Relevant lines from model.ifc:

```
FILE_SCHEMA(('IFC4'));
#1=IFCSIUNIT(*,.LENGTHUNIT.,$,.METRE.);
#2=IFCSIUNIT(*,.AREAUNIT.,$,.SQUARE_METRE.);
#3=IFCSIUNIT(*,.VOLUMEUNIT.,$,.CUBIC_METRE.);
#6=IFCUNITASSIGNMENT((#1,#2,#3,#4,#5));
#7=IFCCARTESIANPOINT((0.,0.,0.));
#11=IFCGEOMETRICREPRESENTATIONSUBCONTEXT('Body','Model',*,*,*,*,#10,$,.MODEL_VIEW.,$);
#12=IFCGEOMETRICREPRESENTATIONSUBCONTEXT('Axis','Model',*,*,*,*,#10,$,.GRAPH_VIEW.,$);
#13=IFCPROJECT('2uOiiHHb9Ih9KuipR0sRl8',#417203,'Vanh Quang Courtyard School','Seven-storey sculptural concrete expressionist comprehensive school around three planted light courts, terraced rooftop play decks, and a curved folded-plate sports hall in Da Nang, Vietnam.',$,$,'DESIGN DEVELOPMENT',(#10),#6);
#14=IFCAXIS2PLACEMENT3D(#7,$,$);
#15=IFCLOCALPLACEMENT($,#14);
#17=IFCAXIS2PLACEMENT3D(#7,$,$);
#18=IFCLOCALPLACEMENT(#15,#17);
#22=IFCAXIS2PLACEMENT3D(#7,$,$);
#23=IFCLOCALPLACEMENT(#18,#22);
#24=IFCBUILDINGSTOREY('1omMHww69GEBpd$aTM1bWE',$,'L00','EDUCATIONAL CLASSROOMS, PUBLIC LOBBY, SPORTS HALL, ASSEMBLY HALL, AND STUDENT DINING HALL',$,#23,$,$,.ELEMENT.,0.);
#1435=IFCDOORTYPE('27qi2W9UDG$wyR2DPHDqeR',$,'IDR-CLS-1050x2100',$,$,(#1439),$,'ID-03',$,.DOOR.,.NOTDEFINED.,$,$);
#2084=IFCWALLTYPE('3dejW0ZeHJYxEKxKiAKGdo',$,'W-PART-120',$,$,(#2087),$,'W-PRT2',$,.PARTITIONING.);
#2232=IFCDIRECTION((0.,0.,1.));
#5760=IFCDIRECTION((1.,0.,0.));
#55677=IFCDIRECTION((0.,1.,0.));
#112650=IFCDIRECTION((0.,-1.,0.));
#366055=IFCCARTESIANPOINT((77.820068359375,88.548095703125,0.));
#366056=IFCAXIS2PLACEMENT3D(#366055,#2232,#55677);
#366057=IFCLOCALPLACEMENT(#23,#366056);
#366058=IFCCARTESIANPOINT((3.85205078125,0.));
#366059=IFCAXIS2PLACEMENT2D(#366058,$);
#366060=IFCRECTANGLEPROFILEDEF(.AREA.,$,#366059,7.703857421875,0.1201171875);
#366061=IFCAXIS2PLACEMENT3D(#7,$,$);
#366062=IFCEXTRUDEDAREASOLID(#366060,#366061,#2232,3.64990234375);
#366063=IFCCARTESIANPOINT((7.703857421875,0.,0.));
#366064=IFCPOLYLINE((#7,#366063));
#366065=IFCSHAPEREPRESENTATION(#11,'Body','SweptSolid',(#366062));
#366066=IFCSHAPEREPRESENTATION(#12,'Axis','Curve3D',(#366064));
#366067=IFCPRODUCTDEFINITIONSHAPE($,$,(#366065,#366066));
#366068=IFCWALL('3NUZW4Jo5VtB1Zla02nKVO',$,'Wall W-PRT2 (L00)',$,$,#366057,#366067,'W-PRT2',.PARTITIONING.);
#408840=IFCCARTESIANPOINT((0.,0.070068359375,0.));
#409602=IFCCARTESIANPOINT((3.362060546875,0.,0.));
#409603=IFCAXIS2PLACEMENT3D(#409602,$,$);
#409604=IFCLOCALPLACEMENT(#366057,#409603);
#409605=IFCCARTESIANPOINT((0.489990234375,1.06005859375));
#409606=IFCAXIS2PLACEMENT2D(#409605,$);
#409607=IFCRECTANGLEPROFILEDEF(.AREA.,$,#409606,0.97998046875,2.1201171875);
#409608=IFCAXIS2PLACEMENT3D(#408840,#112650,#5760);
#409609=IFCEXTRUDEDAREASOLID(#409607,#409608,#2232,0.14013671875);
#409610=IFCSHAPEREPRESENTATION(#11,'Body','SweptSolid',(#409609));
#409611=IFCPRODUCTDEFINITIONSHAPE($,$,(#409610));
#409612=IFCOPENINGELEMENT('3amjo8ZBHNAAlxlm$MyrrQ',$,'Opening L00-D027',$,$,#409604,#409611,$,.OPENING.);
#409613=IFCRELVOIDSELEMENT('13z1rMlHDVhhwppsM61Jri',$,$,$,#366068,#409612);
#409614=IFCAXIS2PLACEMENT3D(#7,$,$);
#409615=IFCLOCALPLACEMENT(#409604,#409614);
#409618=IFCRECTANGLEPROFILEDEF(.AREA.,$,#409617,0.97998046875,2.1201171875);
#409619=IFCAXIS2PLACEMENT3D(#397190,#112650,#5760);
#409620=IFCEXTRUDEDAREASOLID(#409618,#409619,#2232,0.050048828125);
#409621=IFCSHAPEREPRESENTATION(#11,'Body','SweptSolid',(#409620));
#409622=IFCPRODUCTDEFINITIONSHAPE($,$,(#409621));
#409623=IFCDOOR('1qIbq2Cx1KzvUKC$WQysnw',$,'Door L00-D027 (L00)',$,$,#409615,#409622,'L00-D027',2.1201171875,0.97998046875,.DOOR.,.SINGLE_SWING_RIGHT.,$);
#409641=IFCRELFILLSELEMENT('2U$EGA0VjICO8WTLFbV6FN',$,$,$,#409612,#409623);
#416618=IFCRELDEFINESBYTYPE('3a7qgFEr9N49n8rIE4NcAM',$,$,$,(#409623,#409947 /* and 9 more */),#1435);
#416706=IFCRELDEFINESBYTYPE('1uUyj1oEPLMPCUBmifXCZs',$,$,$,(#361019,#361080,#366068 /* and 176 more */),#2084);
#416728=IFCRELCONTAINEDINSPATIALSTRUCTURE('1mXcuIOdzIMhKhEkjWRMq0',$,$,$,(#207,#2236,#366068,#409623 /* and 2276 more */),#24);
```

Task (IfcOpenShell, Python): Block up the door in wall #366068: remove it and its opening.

```python
import ifcopenshell
import ifcopenshell.api.feature
import ifcopenshell.api.root
import ifcopenshell.geom
import ifcopenshell.util.shape

model = ifcopenshell.open("model.ifc")
settings = ifcopenshell.geom.settings()


def volume(element):
    """Net volume in cubic metres, openings subtracted."""
    shape = ifcopenshell.geom.create_shape(settings, element)
    return ifcopenshell.util.shape.get_volume(shape.geometry)


door = model.by_id(409623)
opening = door.FillsVoids[0].RelatingOpeningElement
wall = opening.VoidsElements[0].RelatingBuildingElement
before = volume(wall)

ifcopenshell.api.root.remove_product(model, product=door)
ifcopenshell.api.feature.remove_feature(model, feature=opening)

after = volume(wall)

print(f"wall volume {before:.3f} -> {after:.3f} m3")

model.write("model_rev.ifc")
```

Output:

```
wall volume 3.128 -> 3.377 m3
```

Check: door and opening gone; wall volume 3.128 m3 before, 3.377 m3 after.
